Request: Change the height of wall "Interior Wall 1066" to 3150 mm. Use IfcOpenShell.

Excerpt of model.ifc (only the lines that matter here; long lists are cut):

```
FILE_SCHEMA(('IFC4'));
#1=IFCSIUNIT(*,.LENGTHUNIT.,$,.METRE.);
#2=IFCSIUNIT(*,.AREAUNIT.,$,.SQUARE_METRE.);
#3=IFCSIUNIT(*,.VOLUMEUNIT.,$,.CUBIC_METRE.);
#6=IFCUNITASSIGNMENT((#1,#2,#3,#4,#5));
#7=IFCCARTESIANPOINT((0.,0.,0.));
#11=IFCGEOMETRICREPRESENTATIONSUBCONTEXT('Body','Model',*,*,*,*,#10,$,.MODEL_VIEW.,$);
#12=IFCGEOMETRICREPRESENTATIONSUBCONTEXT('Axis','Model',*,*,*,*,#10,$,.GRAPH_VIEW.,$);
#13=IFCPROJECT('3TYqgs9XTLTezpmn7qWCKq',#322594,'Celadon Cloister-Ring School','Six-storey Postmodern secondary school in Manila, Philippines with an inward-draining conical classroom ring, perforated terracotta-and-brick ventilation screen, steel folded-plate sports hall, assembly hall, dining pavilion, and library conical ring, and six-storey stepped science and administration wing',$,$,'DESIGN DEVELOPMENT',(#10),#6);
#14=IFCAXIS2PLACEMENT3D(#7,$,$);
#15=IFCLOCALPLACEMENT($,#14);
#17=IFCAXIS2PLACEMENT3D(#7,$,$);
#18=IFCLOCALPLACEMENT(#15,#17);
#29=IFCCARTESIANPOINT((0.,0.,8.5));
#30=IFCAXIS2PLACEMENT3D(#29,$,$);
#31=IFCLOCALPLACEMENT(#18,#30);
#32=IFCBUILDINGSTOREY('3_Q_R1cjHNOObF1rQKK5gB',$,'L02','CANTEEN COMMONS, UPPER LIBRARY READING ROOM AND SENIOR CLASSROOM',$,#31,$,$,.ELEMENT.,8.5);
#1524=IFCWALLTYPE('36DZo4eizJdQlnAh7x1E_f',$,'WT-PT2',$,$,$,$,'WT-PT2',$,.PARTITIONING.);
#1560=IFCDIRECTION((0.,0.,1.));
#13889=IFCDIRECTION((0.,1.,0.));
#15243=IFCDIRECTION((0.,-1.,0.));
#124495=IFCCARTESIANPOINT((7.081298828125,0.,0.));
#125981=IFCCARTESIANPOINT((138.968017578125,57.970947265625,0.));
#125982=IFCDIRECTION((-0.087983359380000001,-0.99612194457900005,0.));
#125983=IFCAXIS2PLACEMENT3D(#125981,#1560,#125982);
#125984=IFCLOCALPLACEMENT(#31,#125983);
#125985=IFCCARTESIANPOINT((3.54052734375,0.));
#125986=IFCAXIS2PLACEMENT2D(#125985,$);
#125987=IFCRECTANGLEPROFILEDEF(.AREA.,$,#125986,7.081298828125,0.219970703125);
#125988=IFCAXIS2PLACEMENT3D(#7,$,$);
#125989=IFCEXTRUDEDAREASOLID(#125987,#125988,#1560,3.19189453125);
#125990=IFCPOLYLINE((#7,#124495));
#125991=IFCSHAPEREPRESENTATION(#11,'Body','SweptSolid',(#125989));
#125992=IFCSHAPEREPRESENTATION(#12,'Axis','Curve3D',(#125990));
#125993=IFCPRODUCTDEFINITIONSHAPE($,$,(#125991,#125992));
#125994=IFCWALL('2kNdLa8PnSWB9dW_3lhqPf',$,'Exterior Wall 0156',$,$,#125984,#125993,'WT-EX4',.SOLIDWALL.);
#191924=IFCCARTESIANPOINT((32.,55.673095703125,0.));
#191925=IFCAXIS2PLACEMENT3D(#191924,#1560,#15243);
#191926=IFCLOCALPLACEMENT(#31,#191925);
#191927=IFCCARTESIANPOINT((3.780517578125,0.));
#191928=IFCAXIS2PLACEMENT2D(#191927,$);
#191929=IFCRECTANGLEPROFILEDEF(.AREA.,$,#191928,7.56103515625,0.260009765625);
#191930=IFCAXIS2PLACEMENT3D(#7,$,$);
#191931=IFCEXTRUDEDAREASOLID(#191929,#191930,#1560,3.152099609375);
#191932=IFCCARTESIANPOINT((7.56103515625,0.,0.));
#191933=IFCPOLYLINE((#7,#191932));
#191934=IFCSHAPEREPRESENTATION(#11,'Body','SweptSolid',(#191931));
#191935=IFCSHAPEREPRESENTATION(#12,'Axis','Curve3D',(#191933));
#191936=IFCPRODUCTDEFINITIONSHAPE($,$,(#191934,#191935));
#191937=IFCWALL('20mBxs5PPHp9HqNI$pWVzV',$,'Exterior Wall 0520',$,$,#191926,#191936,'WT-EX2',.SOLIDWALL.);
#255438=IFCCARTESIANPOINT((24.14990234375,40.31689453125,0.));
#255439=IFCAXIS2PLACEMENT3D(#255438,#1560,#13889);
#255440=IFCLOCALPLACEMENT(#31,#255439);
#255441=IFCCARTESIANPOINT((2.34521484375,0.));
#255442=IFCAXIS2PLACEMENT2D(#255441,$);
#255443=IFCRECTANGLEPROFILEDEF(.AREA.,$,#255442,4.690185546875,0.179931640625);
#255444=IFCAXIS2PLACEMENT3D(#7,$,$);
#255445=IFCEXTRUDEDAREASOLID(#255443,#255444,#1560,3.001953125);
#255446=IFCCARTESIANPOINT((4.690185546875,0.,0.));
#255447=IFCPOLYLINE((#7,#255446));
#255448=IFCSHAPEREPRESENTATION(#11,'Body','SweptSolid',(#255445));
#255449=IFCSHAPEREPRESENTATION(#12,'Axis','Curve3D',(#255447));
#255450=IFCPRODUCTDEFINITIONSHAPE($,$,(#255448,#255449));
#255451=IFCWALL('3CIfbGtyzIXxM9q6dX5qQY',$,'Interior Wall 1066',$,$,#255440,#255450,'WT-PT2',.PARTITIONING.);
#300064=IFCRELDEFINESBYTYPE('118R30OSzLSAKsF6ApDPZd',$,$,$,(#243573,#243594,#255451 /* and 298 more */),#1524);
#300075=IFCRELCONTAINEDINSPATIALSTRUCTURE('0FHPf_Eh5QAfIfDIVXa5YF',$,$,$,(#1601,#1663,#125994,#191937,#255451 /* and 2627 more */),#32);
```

```python
import ifcopenshell
import ifcopenshell.geom
import ifcopenshell.util.representation
import ifcopenshell.util.shape

model = ifcopenshell.open("model.ifc")
settings = ifcopenshell.geom.settings()


def volume(element):
    """Net volume in cubic metres, openings subtracted."""
    shape = ifcopenshell.geom.create_shape(settings, element)
    return ifcopenshell.util.shape.get_volume(shape.geometry)


wall = model.by_id(255451)
before = volume(wall)

body = ifcopenshell.util.representation.get_representation(wall, "Model", "Body")
solid = body.Items[0]
old_height = solid.Depth
solid.Depth = 3.15
after = volume(wall)

print(f"height {old_height:g} -> {solid.Depth:g}, volume {before:.3f} -> {after:.3f} m3")

model.write("model-out.ifc")
```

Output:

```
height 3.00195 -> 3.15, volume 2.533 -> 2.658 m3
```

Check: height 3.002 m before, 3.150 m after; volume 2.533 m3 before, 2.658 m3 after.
